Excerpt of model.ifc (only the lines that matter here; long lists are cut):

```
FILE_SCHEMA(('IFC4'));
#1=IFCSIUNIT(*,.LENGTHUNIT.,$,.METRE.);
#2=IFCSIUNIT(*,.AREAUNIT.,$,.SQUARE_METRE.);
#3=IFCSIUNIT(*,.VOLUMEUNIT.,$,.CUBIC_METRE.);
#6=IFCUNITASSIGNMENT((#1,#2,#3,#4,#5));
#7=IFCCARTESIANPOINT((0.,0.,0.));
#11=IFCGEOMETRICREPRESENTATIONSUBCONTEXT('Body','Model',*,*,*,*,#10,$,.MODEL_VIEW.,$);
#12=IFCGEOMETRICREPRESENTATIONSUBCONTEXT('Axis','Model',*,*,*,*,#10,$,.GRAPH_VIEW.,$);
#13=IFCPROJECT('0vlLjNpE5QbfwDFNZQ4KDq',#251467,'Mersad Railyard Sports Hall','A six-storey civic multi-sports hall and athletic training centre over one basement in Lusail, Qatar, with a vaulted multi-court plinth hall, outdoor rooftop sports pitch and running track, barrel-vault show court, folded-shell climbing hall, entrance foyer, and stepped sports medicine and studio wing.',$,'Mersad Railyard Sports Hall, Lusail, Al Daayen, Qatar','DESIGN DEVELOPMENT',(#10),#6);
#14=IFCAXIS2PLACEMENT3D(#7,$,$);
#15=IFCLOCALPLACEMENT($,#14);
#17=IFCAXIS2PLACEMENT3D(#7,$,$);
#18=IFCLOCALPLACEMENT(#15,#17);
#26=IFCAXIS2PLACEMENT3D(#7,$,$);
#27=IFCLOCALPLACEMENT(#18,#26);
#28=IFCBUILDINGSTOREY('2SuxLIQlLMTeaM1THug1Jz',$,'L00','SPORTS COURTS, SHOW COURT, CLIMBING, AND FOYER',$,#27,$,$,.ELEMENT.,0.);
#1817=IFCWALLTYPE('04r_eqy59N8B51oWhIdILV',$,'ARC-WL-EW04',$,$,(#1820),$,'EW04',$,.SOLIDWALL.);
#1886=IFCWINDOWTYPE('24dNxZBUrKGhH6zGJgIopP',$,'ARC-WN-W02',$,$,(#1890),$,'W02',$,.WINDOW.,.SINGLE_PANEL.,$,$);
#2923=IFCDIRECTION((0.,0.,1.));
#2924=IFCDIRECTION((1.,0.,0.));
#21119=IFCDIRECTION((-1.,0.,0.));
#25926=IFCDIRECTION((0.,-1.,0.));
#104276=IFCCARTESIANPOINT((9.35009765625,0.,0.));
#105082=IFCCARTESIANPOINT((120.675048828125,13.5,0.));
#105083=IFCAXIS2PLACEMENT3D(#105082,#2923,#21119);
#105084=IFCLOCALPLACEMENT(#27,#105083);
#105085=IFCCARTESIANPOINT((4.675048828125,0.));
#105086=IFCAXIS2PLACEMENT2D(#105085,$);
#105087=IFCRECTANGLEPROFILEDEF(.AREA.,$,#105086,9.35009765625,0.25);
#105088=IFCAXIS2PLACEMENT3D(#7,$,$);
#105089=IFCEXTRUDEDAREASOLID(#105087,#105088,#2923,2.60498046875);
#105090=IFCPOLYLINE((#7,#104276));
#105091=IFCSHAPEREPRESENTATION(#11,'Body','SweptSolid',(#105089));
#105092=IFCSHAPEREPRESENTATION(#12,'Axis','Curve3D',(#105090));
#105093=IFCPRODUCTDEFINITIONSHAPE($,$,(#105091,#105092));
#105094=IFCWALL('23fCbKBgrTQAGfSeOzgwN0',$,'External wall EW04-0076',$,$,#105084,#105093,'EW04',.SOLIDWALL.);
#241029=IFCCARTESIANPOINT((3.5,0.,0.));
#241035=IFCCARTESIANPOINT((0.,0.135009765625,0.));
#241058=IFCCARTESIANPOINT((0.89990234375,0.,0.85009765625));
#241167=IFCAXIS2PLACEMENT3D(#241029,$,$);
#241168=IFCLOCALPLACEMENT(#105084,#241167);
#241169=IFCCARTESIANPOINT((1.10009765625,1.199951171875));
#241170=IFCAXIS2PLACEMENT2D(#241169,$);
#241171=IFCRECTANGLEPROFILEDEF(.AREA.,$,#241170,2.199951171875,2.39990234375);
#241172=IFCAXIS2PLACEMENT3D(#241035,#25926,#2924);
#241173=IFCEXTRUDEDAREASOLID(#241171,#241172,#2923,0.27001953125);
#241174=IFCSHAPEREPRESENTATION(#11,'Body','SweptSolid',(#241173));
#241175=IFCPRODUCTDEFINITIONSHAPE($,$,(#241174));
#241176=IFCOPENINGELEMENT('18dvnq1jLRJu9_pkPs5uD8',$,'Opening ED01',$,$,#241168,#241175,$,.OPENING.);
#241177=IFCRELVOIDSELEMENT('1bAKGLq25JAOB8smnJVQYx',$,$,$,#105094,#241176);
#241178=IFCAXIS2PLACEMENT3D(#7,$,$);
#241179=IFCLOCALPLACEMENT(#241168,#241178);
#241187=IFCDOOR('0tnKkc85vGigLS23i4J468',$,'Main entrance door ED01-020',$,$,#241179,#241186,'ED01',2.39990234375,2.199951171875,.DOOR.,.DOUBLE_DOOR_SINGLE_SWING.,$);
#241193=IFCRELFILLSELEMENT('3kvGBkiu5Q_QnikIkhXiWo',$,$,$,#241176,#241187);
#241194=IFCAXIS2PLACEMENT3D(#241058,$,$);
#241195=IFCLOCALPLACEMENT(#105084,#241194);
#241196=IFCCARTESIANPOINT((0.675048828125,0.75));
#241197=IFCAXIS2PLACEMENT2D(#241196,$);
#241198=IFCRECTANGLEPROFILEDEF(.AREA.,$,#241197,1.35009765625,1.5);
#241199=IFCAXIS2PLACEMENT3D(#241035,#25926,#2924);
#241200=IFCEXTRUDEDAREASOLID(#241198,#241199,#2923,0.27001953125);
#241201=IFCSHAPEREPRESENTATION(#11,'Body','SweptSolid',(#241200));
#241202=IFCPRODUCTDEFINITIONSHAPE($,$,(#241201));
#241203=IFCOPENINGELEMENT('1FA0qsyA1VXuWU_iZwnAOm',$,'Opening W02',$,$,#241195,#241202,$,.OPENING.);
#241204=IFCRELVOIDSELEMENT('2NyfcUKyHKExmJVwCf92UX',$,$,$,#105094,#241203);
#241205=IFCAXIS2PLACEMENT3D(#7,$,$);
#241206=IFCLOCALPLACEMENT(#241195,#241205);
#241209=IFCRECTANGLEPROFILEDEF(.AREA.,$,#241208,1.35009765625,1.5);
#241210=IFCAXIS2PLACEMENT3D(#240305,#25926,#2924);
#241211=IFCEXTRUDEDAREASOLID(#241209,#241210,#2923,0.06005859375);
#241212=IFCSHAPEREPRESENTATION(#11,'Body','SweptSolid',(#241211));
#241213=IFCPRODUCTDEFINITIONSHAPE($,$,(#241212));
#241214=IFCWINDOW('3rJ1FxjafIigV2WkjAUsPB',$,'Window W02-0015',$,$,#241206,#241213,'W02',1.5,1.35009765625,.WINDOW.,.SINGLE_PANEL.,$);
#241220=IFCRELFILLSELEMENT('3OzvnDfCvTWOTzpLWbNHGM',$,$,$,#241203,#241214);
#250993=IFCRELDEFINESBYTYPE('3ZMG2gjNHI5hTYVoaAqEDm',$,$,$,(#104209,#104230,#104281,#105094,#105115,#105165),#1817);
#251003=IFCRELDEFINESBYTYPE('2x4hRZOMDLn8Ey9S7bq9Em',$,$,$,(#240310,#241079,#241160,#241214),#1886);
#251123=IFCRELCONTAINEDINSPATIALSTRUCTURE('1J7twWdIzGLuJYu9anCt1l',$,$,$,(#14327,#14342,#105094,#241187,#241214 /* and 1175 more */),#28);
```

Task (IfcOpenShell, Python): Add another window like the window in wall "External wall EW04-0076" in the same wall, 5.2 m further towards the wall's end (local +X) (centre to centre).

```python
import ifcopenshell
import ifcopenshell.api.feature
import ifcopenshell.api.geometry
import ifcopenshell.api.root
import ifcopenshell.geom
import ifcopenshell.util.element
import ifcopenshell.util.placement
import ifcopenshell.util.shape

model = ifcopenshell.open("model.ifc")
settings = ifcopenshell.geom.settings()


def volume(element):
    """Net volume in cubic metres, openings subtracted."""
    shape = ifcopenshell.geom.create_shape(settings, element)
    return ifcopenshell.util.shape.get_volume(shape.geometry)


window = model.by_guid("3rJ1FxjafIigV2WkjAUsPB")
opening = window.FillsVoids[0].RelatingOpeningElement
wall = opening.VoidsElements[0].RelatingBuildingElement
before = volume(wall)
shift = ifcopenshell.util.placement.get_local_placement(wall.ObjectPlacement)[:3, 0] * 5.2

# copy_class copies the void relationship, type, container and properties, but no geometry.
new_opening = ifcopenshell.api.root.copy_class(model, product=opening)
new_opening.Representation = ifcopenshell.util.element.copy_deep(
    model, opening.Representation, exclude=["IfcGeometricRepresentationContext", "IfcRepresentationMap"]
)
new_window = ifcopenshell.api.root.copy_class(model, product=window)
new_window.Representation = ifcopenshell.util.element.copy_deep(
    model, window.Representation, exclude=["IfcGeometricRepresentationContext", "IfcRepresentationMap"]
)
new_window.Tag = None
ifcopenshell.api.feature.add_filling(model, opening=new_opening, element=new_window)

for old, new in ((opening, new_opening), (window, new_window)):
    matrix = ifcopenshell.util.placement.get_local_placement(old.ObjectPlacement)
    matrix[:3, 3] += shift
    ifcopenshell.api.geometry.edit_object_placement(model, product=new, matrix=matrix, is_si=False)

after = volume(wall)

print(f"wall volume {before:.3f} -> {after:.3f} m3")

model.write("model_updated.ifc")
```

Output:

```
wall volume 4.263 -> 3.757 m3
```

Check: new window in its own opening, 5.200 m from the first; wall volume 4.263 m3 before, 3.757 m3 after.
